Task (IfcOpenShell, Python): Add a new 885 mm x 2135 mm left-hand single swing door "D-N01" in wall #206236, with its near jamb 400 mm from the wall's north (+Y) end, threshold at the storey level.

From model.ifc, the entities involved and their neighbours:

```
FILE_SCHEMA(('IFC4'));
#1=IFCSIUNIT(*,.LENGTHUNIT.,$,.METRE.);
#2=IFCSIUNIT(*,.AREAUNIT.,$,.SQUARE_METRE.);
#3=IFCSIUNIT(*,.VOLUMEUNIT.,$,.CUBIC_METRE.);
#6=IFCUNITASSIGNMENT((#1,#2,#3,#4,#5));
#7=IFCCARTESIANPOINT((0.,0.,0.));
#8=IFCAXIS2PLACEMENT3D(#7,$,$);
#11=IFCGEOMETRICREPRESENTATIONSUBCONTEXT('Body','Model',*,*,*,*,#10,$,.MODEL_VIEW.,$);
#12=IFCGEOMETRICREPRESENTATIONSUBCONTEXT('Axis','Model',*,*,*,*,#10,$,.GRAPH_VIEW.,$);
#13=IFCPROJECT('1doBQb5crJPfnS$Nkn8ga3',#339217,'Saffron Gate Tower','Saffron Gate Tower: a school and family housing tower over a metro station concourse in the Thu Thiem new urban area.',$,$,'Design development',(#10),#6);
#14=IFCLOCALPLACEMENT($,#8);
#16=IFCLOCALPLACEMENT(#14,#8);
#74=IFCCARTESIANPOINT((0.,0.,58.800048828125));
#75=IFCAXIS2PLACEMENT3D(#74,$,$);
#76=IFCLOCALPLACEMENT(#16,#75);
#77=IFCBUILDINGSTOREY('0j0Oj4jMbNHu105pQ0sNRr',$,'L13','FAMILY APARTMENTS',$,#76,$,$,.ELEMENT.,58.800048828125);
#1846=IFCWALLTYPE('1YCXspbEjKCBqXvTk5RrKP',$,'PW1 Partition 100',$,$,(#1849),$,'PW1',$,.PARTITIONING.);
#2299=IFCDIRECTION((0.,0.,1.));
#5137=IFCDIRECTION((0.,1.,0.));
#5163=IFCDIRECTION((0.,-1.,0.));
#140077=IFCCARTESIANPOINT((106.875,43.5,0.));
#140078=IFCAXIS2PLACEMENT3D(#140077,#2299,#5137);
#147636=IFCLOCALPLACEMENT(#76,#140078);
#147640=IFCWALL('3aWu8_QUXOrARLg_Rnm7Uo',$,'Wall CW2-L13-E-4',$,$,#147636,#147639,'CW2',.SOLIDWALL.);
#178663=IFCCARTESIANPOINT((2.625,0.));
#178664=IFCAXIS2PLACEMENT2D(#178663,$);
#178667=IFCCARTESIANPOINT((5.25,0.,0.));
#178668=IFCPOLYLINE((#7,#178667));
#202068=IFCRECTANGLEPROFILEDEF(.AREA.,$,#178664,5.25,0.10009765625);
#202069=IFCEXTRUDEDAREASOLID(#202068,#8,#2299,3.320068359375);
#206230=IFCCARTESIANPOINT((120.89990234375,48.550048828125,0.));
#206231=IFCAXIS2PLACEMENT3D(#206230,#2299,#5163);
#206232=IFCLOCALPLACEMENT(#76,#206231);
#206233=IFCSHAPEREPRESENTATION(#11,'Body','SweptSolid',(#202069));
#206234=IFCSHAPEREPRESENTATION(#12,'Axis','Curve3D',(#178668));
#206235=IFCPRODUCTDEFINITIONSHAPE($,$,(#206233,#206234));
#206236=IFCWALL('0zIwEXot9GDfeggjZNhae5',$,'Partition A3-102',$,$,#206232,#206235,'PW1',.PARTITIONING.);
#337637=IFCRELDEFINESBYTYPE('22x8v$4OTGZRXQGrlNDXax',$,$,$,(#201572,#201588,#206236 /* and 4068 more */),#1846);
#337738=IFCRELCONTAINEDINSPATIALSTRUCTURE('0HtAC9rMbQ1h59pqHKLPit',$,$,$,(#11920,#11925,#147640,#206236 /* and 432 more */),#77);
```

```python
import numpy as np
import ifcopenshell
import ifcopenshell.api.feature
import ifcopenshell.api.geometry
import ifcopenshell.api.root
import ifcopenshell.api.spatial
import ifcopenshell.geom
import ifcopenshell.util.element
import ifcopenshell.util.placement
import ifcopenshell.util.representation
import ifcopenshell.util.shape
import ifcopenshell.util.unit

model = ifcopenshell.open("model.ifc")
unit_scale = ifcopenshell.util.unit.calculate_unit_scale(model)
settings = ifcopenshell.geom.settings()


def volume(element):
    """Net volume in cubic metres, openings subtracted."""
    shape = ifcopenshell.geom.create_shape(settings, element)
    return ifcopenshell.util.shape.get_volume(shape.geometry)


wall = model.by_id(206236)
storey = ifcopenshell.util.element.get_container(wall, ifc_class="IfcBuildingStorey")
context = ifcopenshell.util.representation.get_context(model, "Model", "Body", "MODEL_VIEW")
before = volume(wall)

width, height, from_end, sill = 0.885, 2.135, 0.4, 0.0  # metres

# The wall runs along its own X axis, and the end named is its -X end.
wall_shape = ifcopenshell.geom.create_shape(settings, wall)
x, y, z = ifcopenshell.util.shape.get_vertices(wall_shape.geometry).T
start = x.min() + from_end
face, thickness = float(y.min()), float(y.max() - y.min())
wall_matrix = ifcopenshell.util.placement.get_local_placement(wall.ObjectPlacement)
level = ifcopenshell.util.placement.get_local_placement(storey.ObjectPlacement)[2, 3]


def in_wall(x, y):
    """Placement at x, y metres in the wall's axes, at sill height."""
    matrix = wall_matrix.copy()
    matrix[:, 3] = wall_matrix @ np.array([x / unit_scale, y / unit_scale, 0.0, 1.0])
    matrix[2, 3] = level + sill / unit_scale
    return matrix


# Opening: a box that overshoots both wall faces by 50 mm.
opening = ifcopenshell.api.root.create_entity(model, ifc_class="IfcOpeningElement", predefined_type="OPENING")
box = ifcopenshell.api.geometry.add_wall_representation(
    model, context=context, length=width, height=height, thickness=thickness + 0.1
)
ifcopenshell.api.geometry.assign_representation(model, product=opening, representation=box)
ifcopenshell.api.geometry.edit_object_placement(model, product=opening, matrix=in_wall(start, face - 0.05), is_si=False)
ifcopenshell.api.feature.add_feature(model, feature=opening, element=wall)

door = ifcopenshell.api.root.create_entity(model, ifc_class="IfcDoor", name="D-N01", predefined_type="DOOR")
door.OverallWidth, door.OverallHeight = width / unit_scale, height / unit_scale
door.OperationType = "SINGLE_SWING_LEFT"
body = ifcopenshell.api.geometry.add_door_representation(
    model,
    context=context,
    overall_width=door.OverallWidth,
    overall_height=door.OverallHeight,
    operation_type="SINGLE_SWING_LEFT",
    lining_properties={"LiningDepth": thickness / unit_scale, "ThresholdDepth": thickness / unit_scale},
)
ifcopenshell.api.geometry.assign_representation(model, product=door, representation=body)
ifcopenshell.api.spatial.assign_container(model, products=[door], relating_structure=storey)
ifcopenshell.api.feature.add_filling(model, opening=opening, element=door)

# The lining spans the wall, so the door starts at the wall face.
ifcopenshell.api.geometry.edit_object_placement(model, product=door, matrix=in_wall(start, face), is_si=False)

after = volume(wall)

print(f"wall volume {before:.3f} -> {after:.3f} m3")

model.write("model_updated.ifc")
```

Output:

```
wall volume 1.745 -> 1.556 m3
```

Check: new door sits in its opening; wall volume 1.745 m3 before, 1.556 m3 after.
